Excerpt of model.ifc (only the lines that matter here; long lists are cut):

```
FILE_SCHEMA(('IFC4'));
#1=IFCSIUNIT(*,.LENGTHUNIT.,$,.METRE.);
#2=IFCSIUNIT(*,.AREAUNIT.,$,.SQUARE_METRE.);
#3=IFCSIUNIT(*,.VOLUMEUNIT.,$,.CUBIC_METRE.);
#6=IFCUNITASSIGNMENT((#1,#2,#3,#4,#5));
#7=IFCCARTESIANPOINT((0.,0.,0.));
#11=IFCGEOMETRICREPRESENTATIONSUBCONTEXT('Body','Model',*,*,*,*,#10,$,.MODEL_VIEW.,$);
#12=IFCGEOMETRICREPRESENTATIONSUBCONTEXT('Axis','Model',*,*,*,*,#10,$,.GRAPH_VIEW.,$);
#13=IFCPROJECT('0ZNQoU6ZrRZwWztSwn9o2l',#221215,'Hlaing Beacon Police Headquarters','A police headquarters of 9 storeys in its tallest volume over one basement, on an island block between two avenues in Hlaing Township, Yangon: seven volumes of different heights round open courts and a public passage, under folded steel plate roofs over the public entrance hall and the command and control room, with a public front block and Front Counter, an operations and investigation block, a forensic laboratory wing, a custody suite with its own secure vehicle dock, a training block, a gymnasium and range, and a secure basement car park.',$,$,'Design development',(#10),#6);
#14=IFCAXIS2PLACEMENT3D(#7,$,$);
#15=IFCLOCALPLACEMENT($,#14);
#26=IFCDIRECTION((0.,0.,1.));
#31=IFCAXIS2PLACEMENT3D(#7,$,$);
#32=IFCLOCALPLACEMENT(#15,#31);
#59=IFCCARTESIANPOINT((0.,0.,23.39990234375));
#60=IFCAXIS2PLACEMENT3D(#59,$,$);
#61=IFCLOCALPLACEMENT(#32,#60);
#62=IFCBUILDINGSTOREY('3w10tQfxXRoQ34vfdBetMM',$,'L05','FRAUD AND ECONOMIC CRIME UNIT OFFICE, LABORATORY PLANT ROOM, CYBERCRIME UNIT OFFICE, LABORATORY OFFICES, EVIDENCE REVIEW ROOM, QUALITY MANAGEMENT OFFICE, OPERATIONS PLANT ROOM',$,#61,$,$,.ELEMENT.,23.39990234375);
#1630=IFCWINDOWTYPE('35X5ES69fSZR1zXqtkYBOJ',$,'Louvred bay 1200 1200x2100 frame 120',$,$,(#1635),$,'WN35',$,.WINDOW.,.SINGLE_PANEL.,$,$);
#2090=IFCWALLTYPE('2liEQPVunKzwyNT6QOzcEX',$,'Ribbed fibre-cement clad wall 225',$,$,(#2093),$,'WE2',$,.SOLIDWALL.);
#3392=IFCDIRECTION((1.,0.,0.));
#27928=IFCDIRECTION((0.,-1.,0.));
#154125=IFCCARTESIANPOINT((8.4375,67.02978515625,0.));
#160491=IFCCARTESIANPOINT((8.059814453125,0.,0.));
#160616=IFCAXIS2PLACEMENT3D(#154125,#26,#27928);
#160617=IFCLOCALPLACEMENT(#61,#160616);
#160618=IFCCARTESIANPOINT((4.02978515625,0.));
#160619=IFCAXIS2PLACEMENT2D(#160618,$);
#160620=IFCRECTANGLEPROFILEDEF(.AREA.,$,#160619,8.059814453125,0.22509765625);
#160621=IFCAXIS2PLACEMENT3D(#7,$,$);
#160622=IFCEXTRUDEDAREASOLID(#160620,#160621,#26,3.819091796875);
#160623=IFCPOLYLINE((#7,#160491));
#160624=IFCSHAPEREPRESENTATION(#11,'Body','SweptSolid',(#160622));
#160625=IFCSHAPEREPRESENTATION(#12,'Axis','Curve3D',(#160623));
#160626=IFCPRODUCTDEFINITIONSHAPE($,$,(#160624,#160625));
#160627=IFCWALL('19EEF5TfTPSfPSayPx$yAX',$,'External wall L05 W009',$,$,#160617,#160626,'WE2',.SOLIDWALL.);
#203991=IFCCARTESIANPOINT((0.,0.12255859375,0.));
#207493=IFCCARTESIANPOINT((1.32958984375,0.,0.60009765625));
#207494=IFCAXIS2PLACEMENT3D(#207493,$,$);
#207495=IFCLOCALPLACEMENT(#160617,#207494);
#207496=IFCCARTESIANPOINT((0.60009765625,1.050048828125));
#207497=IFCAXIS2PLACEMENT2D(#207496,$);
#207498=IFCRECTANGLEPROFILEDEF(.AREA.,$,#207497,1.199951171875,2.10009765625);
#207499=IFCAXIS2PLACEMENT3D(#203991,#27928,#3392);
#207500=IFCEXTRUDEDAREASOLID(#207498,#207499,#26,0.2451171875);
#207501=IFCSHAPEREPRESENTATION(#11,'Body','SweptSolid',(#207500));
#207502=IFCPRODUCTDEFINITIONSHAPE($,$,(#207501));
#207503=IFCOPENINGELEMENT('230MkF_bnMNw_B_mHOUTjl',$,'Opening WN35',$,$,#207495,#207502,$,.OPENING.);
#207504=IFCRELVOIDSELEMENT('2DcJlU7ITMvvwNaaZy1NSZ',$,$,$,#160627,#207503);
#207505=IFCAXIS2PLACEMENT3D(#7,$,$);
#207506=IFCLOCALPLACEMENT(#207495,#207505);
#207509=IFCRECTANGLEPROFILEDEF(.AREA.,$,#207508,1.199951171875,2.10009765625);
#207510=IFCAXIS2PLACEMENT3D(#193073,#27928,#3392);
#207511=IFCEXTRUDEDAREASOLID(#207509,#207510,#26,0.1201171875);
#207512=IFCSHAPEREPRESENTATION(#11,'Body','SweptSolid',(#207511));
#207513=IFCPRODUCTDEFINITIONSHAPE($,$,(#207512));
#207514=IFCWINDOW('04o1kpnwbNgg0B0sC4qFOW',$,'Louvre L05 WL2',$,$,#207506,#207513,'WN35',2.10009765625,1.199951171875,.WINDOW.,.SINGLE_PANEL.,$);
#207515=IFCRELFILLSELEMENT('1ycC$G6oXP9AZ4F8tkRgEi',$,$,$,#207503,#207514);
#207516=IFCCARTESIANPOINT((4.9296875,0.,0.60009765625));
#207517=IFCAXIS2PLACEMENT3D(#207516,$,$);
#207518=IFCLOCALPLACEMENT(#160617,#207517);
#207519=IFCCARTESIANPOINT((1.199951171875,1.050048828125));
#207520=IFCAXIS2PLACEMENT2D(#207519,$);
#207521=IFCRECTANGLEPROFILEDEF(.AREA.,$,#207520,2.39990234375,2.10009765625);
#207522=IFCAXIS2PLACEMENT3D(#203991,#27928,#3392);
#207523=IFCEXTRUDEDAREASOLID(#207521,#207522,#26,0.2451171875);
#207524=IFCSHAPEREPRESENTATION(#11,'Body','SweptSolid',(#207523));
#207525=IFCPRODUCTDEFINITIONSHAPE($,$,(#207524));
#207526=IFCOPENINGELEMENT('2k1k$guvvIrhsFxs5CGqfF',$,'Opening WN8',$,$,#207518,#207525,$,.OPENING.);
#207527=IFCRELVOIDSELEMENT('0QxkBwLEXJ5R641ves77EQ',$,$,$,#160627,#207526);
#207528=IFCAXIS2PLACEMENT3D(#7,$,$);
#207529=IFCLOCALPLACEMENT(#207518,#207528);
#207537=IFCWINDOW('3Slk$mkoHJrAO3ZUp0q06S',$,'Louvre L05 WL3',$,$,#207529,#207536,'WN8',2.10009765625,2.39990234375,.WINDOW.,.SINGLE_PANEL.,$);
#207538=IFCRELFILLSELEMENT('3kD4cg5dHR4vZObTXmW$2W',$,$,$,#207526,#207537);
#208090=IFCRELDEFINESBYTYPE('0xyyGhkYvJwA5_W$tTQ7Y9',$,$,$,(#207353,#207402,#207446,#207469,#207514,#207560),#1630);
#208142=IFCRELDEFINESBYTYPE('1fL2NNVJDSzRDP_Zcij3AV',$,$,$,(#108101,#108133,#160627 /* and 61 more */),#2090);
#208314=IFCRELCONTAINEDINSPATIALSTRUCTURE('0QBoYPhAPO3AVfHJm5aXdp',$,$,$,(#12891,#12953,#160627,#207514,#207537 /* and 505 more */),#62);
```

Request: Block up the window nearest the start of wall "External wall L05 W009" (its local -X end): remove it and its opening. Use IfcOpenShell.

```python
import ifcopenshell
import ifcopenshell.api.feature
import ifcopenshell.api.root
import ifcopenshell.geom
import ifcopenshell.util.shape

model = ifcopenshell.open("model.ifc")
settings = ifcopenshell.geom.settings()


def volume(element):
    """Net volume in cubic metres, openings subtracted."""
    shape = ifcopenshell.geom.create_shape(settings, element)
    return ifcopenshell.util.shape.get_volume(shape.geometry)


window = model.by_id(207514)
opening = window.FillsVoids[0].RelatingOpeningElement
wall = opening.VoidsElements[0].RelatingBuildingElement
before = volume(wall)

ifcopenshell.api.root.remove_product(model, product=window)
ifcopenshell.api.feature.remove_feature(model, feature=opening)

after = volume(wall)

print(f"wall volume {before:.3f} -> {after:.3f} m3")

model.write("model_edited.ifc")
```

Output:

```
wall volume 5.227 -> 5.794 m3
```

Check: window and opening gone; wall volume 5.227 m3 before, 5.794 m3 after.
